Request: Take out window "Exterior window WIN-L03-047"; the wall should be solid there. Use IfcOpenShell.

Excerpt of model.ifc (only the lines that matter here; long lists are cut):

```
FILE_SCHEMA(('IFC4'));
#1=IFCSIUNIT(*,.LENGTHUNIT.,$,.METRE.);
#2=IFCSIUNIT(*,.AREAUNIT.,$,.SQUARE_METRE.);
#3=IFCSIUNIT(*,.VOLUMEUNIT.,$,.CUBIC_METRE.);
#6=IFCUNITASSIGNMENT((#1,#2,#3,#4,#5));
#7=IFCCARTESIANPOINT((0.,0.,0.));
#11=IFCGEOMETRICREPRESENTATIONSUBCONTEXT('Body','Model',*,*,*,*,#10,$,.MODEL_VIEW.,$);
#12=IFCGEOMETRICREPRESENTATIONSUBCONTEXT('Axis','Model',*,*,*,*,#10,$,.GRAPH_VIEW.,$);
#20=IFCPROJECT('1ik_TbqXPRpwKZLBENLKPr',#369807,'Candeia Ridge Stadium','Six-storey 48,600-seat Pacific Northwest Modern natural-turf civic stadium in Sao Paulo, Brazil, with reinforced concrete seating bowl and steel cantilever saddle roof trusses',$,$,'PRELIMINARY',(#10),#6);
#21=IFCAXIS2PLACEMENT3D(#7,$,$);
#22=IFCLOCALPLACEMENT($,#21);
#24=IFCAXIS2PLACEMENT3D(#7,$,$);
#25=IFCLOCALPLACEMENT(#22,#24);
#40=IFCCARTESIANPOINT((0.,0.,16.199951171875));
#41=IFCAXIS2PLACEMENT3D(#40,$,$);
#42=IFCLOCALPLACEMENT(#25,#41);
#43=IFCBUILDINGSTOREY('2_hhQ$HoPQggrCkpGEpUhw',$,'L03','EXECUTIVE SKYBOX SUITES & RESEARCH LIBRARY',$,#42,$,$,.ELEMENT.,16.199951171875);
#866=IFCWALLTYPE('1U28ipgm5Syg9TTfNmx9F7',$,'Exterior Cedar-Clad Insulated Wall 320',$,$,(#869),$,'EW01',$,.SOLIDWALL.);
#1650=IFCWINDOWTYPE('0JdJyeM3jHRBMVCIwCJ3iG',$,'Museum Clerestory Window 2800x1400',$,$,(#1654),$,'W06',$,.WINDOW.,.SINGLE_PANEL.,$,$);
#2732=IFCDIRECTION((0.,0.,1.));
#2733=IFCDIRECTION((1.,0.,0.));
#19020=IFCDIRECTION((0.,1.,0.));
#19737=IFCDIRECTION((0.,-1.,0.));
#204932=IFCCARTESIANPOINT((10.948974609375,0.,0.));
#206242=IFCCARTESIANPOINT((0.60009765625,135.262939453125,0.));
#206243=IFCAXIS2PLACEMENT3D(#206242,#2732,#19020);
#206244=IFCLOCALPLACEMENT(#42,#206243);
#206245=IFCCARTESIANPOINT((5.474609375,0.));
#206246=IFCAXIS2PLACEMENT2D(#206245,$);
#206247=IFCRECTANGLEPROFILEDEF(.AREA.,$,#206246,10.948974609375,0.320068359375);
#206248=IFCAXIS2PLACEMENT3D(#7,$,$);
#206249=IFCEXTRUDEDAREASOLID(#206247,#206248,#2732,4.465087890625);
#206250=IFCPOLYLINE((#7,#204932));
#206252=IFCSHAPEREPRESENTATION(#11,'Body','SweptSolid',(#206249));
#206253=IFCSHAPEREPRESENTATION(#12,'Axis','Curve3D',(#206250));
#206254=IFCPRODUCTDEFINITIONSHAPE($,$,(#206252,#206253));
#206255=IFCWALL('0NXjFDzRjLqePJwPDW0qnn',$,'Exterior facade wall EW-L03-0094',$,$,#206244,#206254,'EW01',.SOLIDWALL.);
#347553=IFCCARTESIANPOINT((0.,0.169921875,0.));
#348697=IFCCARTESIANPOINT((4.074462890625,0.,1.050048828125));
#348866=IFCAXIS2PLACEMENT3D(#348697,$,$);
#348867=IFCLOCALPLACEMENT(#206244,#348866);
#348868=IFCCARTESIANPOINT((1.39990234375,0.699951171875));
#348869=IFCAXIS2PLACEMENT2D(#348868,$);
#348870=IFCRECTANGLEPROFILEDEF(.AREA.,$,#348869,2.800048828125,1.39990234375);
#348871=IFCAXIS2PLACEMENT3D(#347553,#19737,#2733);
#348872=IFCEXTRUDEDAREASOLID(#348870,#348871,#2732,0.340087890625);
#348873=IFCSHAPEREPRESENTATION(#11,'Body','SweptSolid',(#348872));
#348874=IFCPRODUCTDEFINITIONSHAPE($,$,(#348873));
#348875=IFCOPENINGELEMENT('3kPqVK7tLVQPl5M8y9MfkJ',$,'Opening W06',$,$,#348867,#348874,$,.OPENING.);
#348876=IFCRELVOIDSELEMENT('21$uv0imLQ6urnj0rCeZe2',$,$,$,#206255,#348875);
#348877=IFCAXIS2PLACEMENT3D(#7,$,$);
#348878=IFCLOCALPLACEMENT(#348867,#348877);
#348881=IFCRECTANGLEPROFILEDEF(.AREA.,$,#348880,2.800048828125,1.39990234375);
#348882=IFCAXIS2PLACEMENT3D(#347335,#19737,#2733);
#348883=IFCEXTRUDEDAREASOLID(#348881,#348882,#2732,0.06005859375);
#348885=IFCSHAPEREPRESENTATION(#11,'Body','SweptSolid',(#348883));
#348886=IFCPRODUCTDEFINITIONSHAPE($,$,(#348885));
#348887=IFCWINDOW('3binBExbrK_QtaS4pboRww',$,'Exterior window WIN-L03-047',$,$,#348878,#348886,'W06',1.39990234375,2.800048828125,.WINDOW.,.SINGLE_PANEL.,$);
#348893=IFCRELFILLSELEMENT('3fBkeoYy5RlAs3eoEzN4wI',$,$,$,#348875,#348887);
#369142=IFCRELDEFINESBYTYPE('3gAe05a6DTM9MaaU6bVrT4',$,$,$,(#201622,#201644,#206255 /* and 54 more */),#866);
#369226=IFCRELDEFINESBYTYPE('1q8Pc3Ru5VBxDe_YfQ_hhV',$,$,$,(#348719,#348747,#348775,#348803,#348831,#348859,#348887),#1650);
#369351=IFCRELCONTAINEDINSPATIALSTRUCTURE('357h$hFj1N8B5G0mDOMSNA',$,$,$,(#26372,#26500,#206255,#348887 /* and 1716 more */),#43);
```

```python
import ifcopenshell
import ifcopenshell.api.feature
import ifcopenshell.api.root
import ifcopenshell.geom
import ifcopenshell.util.shape

model = ifcopenshell.open("model.ifc")
settings = ifcopenshell.geom.settings()


def volume(element):
    """Net volume in cubic metres, openings subtracted."""
    shape = ifcopenshell.geom.create_shape(settings, element)
    return ifcopenshell.util.shape.get_volume(shape.geometry)


window = model.by_guid("3binBExbrK_QtaS4pboRww")
opening = window.FillsVoids[0].RelatingOpeningElement
wall = opening.VoidsElements[0].RelatingBuildingElement
before = volume(wall)

ifcopenshell.api.root.remove_product(model, product=window)
ifcopenshell.api.feature.remove_feature(model, feature=opening)

after = volume(wall)

print(f"wall volume {before:.3f} -> {after:.3f} m3")

model.write("model_rev.ifc")
```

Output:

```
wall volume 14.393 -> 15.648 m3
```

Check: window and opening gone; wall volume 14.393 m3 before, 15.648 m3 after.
